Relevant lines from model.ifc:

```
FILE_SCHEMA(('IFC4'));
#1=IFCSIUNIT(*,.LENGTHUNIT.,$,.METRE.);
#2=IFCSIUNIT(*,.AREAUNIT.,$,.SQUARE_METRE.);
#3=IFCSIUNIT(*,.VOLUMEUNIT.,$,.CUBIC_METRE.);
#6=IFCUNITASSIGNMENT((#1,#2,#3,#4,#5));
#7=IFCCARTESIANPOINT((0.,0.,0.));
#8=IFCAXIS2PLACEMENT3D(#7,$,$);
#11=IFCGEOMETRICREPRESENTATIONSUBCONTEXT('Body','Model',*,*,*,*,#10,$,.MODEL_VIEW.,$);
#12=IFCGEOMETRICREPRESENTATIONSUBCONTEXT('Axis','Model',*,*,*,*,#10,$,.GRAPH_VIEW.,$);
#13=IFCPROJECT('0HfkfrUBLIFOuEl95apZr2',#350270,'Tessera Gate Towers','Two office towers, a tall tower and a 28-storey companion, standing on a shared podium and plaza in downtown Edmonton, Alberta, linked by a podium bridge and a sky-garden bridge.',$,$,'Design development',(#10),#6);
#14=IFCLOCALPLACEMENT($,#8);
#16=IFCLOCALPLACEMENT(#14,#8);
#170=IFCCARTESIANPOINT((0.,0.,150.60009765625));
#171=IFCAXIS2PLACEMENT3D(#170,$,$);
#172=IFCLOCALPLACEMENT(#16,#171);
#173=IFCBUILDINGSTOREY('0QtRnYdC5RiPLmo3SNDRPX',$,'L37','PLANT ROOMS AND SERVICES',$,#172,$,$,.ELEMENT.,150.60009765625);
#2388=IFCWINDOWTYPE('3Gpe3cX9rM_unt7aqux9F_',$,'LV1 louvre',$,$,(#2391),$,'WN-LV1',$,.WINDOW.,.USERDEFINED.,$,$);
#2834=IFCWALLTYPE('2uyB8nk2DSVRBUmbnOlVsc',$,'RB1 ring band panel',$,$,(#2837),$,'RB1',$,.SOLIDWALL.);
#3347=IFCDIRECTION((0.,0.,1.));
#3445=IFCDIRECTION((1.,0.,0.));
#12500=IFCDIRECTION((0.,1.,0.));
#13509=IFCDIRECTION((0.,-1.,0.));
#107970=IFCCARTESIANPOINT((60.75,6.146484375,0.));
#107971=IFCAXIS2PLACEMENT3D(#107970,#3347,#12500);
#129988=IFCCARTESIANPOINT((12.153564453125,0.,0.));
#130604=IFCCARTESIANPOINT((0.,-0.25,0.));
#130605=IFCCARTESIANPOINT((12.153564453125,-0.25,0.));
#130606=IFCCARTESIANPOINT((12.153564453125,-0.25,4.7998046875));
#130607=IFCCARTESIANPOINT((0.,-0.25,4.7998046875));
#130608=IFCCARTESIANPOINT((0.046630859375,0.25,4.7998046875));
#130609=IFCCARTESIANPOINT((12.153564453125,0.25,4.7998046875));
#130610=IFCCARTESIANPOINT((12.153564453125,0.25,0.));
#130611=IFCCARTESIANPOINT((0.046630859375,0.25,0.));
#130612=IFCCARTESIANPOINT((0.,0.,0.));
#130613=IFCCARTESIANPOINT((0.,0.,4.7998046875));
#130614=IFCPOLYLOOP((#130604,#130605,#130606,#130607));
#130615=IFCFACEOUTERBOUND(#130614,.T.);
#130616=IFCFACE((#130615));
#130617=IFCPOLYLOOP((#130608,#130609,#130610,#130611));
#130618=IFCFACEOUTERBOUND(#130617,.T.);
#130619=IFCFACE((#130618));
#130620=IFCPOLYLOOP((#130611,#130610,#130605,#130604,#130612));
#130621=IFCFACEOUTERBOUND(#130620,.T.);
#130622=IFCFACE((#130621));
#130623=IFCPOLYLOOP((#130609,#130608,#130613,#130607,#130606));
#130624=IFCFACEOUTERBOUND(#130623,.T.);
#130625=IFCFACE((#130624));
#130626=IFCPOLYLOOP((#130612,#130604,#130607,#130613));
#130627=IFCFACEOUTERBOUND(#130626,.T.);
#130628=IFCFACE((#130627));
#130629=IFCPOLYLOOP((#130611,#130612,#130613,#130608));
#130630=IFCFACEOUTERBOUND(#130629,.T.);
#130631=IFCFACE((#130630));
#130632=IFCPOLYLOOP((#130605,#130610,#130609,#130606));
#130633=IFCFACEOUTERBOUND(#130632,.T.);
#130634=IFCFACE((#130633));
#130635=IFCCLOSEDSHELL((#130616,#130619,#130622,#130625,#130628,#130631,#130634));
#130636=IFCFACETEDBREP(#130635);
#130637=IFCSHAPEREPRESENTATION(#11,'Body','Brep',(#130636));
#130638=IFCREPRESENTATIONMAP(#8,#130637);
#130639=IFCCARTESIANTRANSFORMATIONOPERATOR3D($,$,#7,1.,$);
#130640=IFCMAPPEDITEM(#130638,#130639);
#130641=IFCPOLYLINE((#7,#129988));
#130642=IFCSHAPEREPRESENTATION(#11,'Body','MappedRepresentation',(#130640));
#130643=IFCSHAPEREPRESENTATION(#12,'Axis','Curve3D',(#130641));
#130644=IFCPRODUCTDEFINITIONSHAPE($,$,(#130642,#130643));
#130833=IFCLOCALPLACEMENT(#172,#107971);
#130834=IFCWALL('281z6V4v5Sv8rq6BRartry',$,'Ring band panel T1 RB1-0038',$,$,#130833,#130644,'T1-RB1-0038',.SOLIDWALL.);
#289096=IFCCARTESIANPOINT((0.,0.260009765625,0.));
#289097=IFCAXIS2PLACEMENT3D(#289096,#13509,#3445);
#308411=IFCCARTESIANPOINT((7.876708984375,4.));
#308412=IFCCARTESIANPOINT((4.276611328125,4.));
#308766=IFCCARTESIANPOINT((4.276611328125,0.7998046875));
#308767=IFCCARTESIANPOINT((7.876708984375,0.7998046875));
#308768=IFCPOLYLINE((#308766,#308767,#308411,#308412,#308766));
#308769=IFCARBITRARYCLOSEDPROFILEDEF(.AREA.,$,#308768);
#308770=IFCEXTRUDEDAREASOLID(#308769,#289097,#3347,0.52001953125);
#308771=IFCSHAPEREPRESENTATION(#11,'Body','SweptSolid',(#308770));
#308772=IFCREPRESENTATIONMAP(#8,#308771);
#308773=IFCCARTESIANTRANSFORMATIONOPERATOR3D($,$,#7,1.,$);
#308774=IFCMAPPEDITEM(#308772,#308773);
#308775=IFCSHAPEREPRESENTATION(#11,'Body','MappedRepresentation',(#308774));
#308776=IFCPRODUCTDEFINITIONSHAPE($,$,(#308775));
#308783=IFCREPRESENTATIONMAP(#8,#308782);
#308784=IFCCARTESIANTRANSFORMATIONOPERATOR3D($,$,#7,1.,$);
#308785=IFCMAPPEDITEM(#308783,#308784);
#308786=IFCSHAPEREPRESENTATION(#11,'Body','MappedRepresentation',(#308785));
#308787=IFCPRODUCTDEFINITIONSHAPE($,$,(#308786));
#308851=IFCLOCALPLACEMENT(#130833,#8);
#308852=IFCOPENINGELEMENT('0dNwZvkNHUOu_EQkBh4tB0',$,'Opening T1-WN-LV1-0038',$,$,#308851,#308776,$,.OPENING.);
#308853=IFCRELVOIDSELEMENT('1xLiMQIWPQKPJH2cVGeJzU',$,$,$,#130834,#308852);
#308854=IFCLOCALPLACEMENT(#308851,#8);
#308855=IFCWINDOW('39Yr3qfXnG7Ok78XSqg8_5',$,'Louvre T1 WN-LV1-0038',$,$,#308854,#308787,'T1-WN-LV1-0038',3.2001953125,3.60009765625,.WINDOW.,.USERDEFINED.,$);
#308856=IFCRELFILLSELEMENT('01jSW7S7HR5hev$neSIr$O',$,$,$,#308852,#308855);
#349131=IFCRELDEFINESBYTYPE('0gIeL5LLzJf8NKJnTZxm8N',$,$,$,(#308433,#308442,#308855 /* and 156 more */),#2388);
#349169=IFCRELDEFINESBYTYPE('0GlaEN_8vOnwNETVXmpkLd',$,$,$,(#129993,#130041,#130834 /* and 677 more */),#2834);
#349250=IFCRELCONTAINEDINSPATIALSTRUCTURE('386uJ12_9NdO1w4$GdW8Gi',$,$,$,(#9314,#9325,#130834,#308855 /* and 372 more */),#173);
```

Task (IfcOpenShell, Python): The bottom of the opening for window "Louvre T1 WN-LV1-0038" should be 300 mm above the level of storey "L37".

```python
import numpy as np
import ifcopenshell
import ifcopenshell.api.geometry
import ifcopenshell.geom
import ifcopenshell.util.element
import ifcopenshell.util.placement
import ifcopenshell.util.shape
import ifcopenshell.util.unit

model = ifcopenshell.open("model.ifc")
unit_scale = ifcopenshell.util.unit.calculate_unit_scale(model)

window = model.by_guid("39Yr3qfXnG7Ok78XSqg8_5")
opening = window.FillsVoids[0].RelatingOpeningElement
storey = ifcopenshell.util.element.get_container(window, ifc_class="IfcBuildingStorey")
level = ifcopenshell.util.placement.get_local_placement(storey.ObjectPlacement)[2, 3]

# The opening's origin need not be at the sill, so measure its lowest point.
shape = ifcopenshell.geom.create_shape(ifcopenshell.geom.settings(), opening)
bottom = ifcopenshell.util.shape.get_shape_bottom_elevation(shape, shape.geometry) / unit_scale
dz = level + 0.3 / unit_scale - bottom

shift = np.array([0.0, 0.0, dz])
# The window is placed relative to its opening, so it follows when the opening moves.
matrix = ifcopenshell.util.placement.get_local_placement(opening.ObjectPlacement)
matrix[:3, 3] += shift
ifcopenshell.api.geometry.edit_object_placement(
    model, product=opening, matrix=matrix, is_si=False, should_transform_children=True
)

print(f"moved by {dz * unit_scale:+.3f} m")

model.write("model_v2.ifc")
```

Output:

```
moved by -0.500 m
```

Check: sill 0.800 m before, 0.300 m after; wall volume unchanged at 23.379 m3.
